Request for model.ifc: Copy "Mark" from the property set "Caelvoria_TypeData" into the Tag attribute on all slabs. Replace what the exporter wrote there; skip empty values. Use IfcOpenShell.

First a look at what the model holds.

```python
import ifcopenshell
import ifcopenshell.util.element

model = ifcopenshell.open("model.ifc")
print(model.schema)
slabs = model.by_type("IfcSlab")
print(len(slabs), "slabs")
for e in slabs[:8]:
    source = ifcopenshell.util.element.get_pset(e, "Caelvoria_TypeData", "Mark")
    target = e.Tag
    print(e.id(), repr(source), repr(target), sep=" | ")
```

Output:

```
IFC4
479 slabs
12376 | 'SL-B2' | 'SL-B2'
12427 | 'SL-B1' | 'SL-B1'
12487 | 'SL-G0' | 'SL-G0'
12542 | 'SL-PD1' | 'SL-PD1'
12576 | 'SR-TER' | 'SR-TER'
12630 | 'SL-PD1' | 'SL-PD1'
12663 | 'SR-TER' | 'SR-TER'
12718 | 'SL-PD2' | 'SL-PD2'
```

```python
import ifcopenshell
import ifcopenshell.util.element

model = ifcopenshell.open("model.ifc")

count = 0
for e in model.by_type("IfcSlab"):
    value = ifcopenshell.util.element.get_pset(e, "Caelvoria_TypeData", "Mark")
    current = e.Tag
    if not value or not value.strip() or current == value:
        continue
    e.Tag = value
    count += 1

print(count, "slabs updated")

model.write("model_rev.ifc")
```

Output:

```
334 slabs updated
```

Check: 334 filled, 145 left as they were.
